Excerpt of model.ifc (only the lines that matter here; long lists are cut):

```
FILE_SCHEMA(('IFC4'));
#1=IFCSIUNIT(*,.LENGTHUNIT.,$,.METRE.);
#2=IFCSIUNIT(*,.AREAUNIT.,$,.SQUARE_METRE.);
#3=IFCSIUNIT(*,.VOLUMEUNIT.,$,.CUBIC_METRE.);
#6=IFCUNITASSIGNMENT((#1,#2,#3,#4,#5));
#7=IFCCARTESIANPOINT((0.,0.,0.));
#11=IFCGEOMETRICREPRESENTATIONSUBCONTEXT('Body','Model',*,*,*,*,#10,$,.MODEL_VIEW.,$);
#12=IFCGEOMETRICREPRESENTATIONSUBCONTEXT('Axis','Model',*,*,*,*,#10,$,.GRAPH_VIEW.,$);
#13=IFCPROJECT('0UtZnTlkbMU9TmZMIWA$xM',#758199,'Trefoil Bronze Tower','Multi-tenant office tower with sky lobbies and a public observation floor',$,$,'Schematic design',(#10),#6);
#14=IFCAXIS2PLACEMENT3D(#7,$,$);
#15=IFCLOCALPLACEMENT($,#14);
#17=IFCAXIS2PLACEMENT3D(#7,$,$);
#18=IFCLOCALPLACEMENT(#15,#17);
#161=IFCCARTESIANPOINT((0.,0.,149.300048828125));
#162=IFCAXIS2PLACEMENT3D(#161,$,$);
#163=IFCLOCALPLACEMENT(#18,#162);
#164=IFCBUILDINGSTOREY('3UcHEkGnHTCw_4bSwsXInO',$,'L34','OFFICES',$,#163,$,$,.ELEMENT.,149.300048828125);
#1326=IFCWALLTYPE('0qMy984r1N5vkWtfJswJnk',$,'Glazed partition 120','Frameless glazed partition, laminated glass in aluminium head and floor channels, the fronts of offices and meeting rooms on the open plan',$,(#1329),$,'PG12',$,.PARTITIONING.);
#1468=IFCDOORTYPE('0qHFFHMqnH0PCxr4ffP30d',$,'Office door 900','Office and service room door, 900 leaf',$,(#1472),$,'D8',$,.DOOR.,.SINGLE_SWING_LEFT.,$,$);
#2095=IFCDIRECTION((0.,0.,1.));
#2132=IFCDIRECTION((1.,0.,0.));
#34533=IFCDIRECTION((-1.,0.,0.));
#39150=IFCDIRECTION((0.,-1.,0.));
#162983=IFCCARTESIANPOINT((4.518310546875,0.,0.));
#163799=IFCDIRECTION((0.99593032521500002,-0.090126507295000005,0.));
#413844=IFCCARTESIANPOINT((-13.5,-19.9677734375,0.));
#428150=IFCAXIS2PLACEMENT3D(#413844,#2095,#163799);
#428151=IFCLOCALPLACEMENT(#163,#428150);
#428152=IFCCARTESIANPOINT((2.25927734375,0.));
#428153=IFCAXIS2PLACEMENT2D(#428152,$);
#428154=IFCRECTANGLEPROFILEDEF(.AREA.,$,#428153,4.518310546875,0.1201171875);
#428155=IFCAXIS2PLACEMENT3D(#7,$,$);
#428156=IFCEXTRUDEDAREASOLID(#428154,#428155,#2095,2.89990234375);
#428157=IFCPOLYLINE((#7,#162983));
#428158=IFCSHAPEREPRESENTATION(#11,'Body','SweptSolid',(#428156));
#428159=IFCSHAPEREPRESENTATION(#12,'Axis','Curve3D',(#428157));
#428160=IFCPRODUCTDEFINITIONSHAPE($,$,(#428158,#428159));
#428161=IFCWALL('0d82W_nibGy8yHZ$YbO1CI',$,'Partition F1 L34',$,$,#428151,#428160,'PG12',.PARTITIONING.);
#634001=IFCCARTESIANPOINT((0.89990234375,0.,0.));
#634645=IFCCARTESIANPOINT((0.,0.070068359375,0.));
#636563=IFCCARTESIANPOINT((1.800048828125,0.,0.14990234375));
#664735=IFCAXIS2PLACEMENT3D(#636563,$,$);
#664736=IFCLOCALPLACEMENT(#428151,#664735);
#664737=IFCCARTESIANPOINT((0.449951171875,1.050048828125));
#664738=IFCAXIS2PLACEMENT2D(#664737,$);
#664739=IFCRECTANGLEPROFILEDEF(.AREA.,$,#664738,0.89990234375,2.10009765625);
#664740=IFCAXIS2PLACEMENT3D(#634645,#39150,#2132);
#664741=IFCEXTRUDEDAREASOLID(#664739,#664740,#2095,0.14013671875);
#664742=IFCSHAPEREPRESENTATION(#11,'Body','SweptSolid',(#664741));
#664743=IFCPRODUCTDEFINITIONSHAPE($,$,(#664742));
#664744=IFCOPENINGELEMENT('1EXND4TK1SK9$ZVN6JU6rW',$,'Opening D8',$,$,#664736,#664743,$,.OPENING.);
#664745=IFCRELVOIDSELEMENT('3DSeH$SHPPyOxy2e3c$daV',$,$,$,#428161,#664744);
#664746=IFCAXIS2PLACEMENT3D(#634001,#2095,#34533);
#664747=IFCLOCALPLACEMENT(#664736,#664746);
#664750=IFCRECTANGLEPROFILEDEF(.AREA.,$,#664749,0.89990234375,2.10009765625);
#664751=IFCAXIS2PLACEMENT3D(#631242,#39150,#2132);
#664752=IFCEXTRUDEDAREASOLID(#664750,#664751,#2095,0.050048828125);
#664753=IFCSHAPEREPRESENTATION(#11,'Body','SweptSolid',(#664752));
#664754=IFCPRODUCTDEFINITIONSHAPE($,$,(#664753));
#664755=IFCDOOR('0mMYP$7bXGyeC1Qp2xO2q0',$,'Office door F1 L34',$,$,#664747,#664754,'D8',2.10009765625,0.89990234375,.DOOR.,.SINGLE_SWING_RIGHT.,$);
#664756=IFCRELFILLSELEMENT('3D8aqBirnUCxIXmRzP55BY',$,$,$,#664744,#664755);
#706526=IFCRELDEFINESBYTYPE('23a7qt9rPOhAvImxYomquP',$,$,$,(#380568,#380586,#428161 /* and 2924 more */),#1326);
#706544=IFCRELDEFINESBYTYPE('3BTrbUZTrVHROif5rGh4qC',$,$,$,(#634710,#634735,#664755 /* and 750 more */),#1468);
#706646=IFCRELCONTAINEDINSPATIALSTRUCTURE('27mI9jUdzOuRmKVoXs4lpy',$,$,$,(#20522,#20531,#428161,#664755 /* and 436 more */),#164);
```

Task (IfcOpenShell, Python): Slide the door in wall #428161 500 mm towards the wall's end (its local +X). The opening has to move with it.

```python
import ifcopenshell
import ifcopenshell.api.geometry
import ifcopenshell.util.placement

model = ifcopenshell.open("model.ifc")

door = model.by_guid("0mMYP$7bXGyeC1Qp2xO2q0")
opening = door.FillsVoids[0].RelatingOpeningElement
wall = opening.VoidsElements[0].RelatingBuildingElement

wall_matrix = ifcopenshell.util.placement.get_local_placement(wall.ObjectPlacement)
shift = wall_matrix[:3, 0] * 0.5
before = ifcopenshell.util.placement.get_local_placement(door.ObjectPlacement)[:3, 3].copy()

# The door is placed relative to its opening, so it follows when the opening moves.
matrix = ifcopenshell.util.placement.get_local_placement(opening.ObjectPlacement)
matrix[:3, 3] += shift
ifcopenshell.api.geometry.edit_object_placement(
    model, product=opening, matrix=matrix, is_si=False, should_transform_children=True
)

after = ifcopenshell.util.placement.get_local_placement(door.ObjectPlacement)[:3, 3]
print("door moved by", (after - before).round(3) + 0.0)

model.write("model_rev.ifc")
```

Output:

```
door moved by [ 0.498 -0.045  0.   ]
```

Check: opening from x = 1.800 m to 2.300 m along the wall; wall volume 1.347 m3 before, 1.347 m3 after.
